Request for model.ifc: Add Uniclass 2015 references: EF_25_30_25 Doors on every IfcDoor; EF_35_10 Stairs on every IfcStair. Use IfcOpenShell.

First a look at what the model holds.

```python
import ifcopenshell

model = ifcopenshell.open("model.ifc")
print(model.schema)
print("classifications:", [c.Name for c in model.by_type("IfcClassification")])
for ifc_class in ("IfcDoor", "IfcRoof", "IfcStair", "IfcWall", "IfcWindow"):
    print(ifc_class, len(model.by_type(ifc_class)))
```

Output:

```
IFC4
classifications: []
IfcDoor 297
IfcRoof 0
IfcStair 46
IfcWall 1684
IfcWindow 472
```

```python
import ifcopenshell
import ifcopenshell.api.classification

model = ifcopenshell.open("model.ifc")

system = ifcopenshell.api.classification.add_classification(model, classification="Uniclass 2015")

codes = {
    "IfcDoor": ("EF_25_30_25", "Doors"),
    "IfcStair": ("EF_35_10", "Stairs"),
}
for ifc_class, (code, name) in codes.items():
    products = model.by_type(ifc_class)
    ifcopenshell.api.classification.add_reference(
        model, products=products, classification=system, identification=code, name=name
    )
    print(code, len(products))

model.write("model_v2.ifc")
```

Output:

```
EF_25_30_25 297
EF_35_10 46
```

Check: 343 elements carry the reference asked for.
